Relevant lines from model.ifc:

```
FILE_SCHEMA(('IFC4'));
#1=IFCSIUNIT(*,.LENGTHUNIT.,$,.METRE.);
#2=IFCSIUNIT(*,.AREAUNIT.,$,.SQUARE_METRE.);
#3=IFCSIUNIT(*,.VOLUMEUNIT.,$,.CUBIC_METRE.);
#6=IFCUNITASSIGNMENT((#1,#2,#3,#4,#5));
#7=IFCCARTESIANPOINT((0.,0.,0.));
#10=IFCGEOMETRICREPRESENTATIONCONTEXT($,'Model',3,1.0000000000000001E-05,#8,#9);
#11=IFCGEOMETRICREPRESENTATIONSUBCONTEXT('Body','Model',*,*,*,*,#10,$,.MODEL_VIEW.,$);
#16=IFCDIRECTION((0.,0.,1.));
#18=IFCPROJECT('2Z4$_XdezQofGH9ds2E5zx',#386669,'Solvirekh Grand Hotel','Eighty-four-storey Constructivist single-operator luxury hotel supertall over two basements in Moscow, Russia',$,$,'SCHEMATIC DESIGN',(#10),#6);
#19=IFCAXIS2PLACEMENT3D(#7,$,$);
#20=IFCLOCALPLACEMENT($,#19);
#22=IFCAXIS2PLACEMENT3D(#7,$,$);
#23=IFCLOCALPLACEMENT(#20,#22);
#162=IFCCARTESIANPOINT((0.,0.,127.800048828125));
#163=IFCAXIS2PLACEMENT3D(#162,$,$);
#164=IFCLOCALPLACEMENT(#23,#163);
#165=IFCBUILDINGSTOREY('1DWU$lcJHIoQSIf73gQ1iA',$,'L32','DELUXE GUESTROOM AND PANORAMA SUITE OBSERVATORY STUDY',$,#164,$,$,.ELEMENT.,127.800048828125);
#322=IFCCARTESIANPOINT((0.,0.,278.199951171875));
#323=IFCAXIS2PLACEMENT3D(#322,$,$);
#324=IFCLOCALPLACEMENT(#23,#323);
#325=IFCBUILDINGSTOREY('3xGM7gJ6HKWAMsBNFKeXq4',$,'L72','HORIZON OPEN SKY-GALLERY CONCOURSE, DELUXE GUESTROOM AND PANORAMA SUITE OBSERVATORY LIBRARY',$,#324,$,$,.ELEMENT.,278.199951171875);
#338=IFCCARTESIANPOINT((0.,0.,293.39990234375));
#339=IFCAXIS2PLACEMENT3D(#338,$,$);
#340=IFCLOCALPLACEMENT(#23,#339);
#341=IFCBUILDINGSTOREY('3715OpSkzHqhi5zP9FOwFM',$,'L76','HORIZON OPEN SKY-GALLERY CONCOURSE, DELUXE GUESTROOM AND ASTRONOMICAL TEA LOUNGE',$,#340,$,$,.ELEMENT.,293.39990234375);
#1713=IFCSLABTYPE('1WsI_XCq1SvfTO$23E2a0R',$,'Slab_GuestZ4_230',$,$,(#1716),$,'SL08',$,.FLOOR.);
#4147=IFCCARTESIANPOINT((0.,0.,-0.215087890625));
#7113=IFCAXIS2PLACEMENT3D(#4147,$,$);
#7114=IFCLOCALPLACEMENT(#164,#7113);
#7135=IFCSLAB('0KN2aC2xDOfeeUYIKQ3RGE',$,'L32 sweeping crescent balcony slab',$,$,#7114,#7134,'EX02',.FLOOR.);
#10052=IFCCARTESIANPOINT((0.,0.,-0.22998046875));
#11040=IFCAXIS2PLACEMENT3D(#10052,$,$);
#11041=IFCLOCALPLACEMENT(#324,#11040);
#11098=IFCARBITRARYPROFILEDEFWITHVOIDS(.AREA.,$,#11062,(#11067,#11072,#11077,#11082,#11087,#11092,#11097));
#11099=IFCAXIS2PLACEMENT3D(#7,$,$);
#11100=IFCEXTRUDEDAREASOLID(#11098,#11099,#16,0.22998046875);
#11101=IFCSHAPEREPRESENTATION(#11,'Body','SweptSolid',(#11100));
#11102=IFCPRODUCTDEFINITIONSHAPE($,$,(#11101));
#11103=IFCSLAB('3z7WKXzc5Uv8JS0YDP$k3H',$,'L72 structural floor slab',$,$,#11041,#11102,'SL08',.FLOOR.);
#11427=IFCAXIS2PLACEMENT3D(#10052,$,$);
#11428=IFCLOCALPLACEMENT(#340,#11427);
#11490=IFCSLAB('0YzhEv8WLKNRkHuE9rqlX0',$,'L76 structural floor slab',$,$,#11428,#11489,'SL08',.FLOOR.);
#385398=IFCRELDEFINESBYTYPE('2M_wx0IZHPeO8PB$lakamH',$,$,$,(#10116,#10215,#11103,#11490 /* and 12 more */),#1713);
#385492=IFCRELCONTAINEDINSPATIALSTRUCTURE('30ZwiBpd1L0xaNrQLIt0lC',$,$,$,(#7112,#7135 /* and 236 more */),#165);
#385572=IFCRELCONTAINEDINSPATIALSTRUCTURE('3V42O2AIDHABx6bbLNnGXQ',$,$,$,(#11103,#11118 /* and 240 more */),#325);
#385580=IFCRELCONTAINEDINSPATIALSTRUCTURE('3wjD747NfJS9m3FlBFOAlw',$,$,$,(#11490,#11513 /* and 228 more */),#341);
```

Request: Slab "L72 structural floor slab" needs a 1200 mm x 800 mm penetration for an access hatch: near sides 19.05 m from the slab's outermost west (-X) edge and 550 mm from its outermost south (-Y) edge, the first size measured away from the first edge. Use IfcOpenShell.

```python
import numpy as np
import ifcopenshell
import ifcopenshell.api.feature
import ifcopenshell.api.geometry
import ifcopenshell.api.root
import ifcopenshell.geom
import ifcopenshell.util.placement
import ifcopenshell.util.representation
import ifcopenshell.util.shape
import ifcopenshell.util.unit

model = ifcopenshell.open("model.ifc")
unit_scale = ifcopenshell.util.unit.calculate_unit_scale(model)
settings = ifcopenshell.geom.settings()


def volume(element):
    """Net volume in cubic metres, openings subtracted."""
    shape = ifcopenshell.geom.create_shape(settings, element)
    return ifcopenshell.util.shape.get_volume(shape.geometry)


slab = model.by_guid("3z7WKXzc5Uv8JS0YDP$k3H")
before = volume(slab)

# Extent in the slab's own axes, in metres. The edges named are its -X and -Y sides.
slab_shape = ifcopenshell.geom.create_shape(settings, slab)
vertices = ifcopenshell.util.shape.get_vertices(slab_shape.geometry)
x_min, y_min, bottom = vertices.min(axis=0)
top = vertices[:, 2].max()

opening = ifcopenshell.api.root.create_entity(model, ifc_class="IfcOpeningElement", name="Access hatch opening", predefined_type="OPENING")
context = ifcopenshell.util.representation.get_context(model, "Model", "Body", "MODEL_VIEW")
width, depth = 1.2, 0.8
outline = [(0.0, 0.0), (width, 0.0), (width, depth), (0.0, depth), (0.0, 0.0)]
# Overshoot both faces by 50 mm so the cut is clean.
shape = ifcopenshell.api.geometry.add_slab_representation(
    model, context=context, depth=top - bottom + 0.1, polyline=outline
)
ifcopenshell.api.geometry.assign_representation(model, product=opening, representation=shape)

matrix = ifcopenshell.util.placement.get_local_placement(slab.ObjectPlacement)
matrix[:, 3] = matrix @ np.append(np.array([x_min + 19.05, y_min + 0.55, bottom - 0.05]) / unit_scale, 1.0)
ifcopenshell.api.geometry.edit_object_placement(model, product=opening, matrix=matrix, is_si=False)
ifcopenshell.api.feature.add_feature(model, feature=opening, element=slab)

after = volume(slab)

print(f"slab volume {before:.3f} -> {after:.3f} m3")

model.write("model-out.ifc")
```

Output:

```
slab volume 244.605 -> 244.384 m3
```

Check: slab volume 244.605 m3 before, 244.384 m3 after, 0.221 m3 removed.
